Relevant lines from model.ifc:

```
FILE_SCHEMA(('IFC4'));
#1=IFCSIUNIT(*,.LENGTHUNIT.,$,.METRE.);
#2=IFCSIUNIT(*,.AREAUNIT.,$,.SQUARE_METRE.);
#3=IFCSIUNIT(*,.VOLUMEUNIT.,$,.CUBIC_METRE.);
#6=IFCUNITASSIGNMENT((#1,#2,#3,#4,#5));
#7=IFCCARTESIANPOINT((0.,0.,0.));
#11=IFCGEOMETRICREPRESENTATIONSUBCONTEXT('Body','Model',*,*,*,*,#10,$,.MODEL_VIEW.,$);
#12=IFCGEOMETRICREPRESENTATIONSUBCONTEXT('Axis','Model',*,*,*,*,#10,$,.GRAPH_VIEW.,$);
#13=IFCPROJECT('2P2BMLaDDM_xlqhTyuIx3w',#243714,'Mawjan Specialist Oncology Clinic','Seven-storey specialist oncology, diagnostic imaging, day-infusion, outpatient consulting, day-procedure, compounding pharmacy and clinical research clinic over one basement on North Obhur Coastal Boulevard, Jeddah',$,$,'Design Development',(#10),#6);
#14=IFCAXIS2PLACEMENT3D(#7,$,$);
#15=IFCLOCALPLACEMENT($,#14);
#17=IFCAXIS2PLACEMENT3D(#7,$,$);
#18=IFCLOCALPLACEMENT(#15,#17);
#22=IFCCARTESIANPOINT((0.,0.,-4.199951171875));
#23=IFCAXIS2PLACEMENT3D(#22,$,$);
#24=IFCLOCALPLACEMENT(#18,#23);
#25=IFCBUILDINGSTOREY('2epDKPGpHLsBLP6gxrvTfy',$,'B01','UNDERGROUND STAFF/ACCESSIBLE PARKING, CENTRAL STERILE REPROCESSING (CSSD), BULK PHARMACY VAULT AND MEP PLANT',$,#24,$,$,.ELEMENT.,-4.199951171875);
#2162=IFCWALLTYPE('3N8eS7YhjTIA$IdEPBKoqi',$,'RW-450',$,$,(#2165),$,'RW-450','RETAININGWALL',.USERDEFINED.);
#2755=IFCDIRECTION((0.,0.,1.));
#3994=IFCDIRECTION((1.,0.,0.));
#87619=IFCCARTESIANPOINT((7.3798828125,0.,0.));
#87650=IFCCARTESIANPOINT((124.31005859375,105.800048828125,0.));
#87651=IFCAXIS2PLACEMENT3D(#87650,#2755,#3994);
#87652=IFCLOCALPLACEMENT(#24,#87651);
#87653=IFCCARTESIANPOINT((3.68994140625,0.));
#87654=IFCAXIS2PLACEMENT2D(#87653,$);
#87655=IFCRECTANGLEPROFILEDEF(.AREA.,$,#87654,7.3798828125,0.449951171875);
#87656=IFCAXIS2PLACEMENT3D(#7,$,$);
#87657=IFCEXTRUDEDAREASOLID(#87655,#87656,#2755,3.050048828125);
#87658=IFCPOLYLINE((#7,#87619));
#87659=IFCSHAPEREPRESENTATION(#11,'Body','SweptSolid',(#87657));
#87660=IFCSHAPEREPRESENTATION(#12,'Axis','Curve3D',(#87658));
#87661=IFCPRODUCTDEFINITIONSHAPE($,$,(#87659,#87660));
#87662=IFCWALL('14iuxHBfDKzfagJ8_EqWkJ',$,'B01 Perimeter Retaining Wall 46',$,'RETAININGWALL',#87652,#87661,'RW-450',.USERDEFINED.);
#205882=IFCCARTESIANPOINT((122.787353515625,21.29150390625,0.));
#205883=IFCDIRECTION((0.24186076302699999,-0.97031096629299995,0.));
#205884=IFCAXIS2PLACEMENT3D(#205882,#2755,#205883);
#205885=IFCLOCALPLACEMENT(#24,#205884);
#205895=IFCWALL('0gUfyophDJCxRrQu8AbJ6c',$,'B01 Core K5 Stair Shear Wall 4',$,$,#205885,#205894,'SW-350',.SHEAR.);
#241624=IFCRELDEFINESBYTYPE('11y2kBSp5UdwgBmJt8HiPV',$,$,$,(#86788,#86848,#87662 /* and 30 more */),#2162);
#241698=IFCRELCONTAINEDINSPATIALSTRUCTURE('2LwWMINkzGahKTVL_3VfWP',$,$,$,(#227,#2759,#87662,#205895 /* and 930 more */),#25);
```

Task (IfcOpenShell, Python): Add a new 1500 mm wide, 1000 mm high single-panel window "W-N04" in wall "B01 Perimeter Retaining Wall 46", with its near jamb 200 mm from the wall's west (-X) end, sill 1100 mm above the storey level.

```python
import numpy as np
import ifcopenshell
import ifcopenshell.api.feature
import ifcopenshell.api.geometry
import ifcopenshell.api.root
import ifcopenshell.api.spatial
import ifcopenshell.geom
import ifcopenshell.util.element
import ifcopenshell.util.placement
import ifcopenshell.util.representation
import ifcopenshell.util.shape
import ifcopenshell.util.unit

model = ifcopenshell.open("model.ifc")
unit_scale = ifcopenshell.util.unit.calculate_unit_scale(model)
settings = ifcopenshell.geom.settings()


def volume(element):
    """Net volume in cubic metres, openings subtracted."""
    shape = ifcopenshell.geom.create_shape(settings, element)
    return ifcopenshell.util.shape.get_volume(shape.geometry)


wall = model.by_guid("14iuxHBfDKzfagJ8_EqWkJ")
storey = ifcopenshell.util.element.get_container(wall, ifc_class="IfcBuildingStorey")
context = ifcopenshell.util.representation.get_context(model, "Model", "Body", "MODEL_VIEW")
before = volume(wall)

width, height, from_end, sill = 1.5, 1, 0.2, 1.1  # metres

# The wall runs along its own X axis, and the end named is its -X end.
wall_shape = ifcopenshell.geom.create_shape(settings, wall)
x, y, z = ifcopenshell.util.shape.get_vertices(wall_shape.geometry).T
start = x.min() + from_end
face, thickness = float(y.min()), float(y.max() - y.min())
wall_matrix = ifcopenshell.util.placement.get_local_placement(wall.ObjectPlacement)
level = ifcopenshell.util.placement.get_local_placement(storey.ObjectPlacement)[2, 3]


def in_wall(x, y):
    """Placement at x, y metres in the wall's axes, at sill height."""
    matrix = wall_matrix.copy()
    matrix[:, 3] = wall_matrix @ np.array([x / unit_scale, y / unit_scale, 0.0, 1.0])
    matrix[2, 3] = level + sill / unit_scale
    return matrix


# Opening: a box that overshoots both wall faces by 50 mm.
opening = ifcopenshell.api.root.create_entity(model, ifc_class="IfcOpeningElement", predefined_type="OPENING")
box = ifcopenshell.api.geometry.add_wall_representation(
    model, context=context, length=width, height=height, thickness=thickness + 0.1
)
ifcopenshell.api.geometry.assign_representation(model, product=opening, representation=box)
ifcopenshell.api.geometry.edit_object_placement(model, product=opening, matrix=in_wall(start, face - 0.05), is_si=False)
ifcopenshell.api.feature.add_feature(model, feature=opening, element=wall)

window = ifcopenshell.api.root.create_entity(model, ifc_class="IfcWindow", name="W-N04", predefined_type="WINDOW")
window.OverallWidth, window.OverallHeight = width / unit_scale, height / unit_scale
window.PartitioningType = "SINGLE_PANEL"
body = ifcopenshell.api.geometry.add_window_representation(
    model,
    context=context,
    overall_width=window.OverallWidth,
    overall_height=window.OverallHeight,
    partition_type="SINGLE_PANEL",
)
ifcopenshell.api.geometry.assign_representation(model, product=window, representation=body)
ifcopenshell.api.spatial.assign_container(model, products=[window], relating_structure=storey)
ifcopenshell.api.feature.add_filling(model, opening=opening, element=window)

# Centre the window in the wall's thickness.
ifcopenshell.api.geometry.edit_object_placement(model, product=window, matrix=in_wall(start, face), is_si=False)
window_shape = ifcopenshell.geom.create_shape(settings, window)
depth = ifcopenshell.util.shape.get_vertices(window_shape.geometry)[:, 1]
offset = face + thickness / 2 - (depth.min() + depth.max()) / 2
ifcopenshell.api.geometry.edit_object_placement(model, product=window, matrix=in_wall(start, offset), is_si=False)

after = volume(wall)

print(f"wall volume {before:.3f} -> {after:.3f} m3")

model.write("model_v2.ifc")
```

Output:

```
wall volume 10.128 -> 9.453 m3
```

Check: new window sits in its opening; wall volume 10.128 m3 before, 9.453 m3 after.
